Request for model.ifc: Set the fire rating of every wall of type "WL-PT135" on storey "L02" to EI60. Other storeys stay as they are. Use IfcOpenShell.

First a look at what the model holds.

```python
import ifcopenshell
import ifcopenshell.util.element

model = ifcopenshell.open("model.ifc")
print(model.schema)
storey = next(s for s in model.by_type("IfcBuildingStorey") if s.Name == "L02")
walls = [e for e in ifcopenshell.util.element.get_decomposition(storey) if e.is_a("IfcWall")]
seen = {}
for e in walls:
    element_type = ifcopenshell.util.element.get_type(e)
    key = (element_type.Name if element_type != e and element_type else None, ifcopenshell.util.element.get_pset(e, "Pset_WallCommon", "FireRating"))
    seen[key] = seen.get(key, 0) + 1
for (name, value), count in sorted(seen.items(), key=str):
    print(count, "x", name, "|", value)
```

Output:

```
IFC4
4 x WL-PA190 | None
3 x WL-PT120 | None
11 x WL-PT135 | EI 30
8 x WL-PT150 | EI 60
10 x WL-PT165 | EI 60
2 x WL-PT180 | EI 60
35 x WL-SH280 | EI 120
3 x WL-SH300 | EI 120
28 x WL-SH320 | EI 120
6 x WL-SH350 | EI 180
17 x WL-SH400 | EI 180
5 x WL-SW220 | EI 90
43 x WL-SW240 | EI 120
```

```python
import ifcopenshell
import ifcopenshell.api.pset
import ifcopenshell.util.element

model = ifcopenshell.open("model.ifc")

storey = next(s for s in model.by_type("IfcBuildingStorey") if s.Name == "L02")
walls = [e for e in ifcopenshell.util.element.get_decomposition(storey) if e.is_a("IfcWall")]

count = 0
for e in walls:
    element_type = ifcopenshell.util.element.get_type(e)
    if element_type in (None, e) or element_type.Name != "WL-PT135":
        continue
    # add_pset returns the element's existing set when there is one.
    pset = ifcopenshell.api.pset.add_pset(model, product=e, name="Pset_WallCommon")
    ifcopenshell.api.pset.edit_pset(model, pset=pset, properties={"FireRating": "EI60"})
    count += 1

print(count, "walls updated")

model.write("model_v2.ifc")
```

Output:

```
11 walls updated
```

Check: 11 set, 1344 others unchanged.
